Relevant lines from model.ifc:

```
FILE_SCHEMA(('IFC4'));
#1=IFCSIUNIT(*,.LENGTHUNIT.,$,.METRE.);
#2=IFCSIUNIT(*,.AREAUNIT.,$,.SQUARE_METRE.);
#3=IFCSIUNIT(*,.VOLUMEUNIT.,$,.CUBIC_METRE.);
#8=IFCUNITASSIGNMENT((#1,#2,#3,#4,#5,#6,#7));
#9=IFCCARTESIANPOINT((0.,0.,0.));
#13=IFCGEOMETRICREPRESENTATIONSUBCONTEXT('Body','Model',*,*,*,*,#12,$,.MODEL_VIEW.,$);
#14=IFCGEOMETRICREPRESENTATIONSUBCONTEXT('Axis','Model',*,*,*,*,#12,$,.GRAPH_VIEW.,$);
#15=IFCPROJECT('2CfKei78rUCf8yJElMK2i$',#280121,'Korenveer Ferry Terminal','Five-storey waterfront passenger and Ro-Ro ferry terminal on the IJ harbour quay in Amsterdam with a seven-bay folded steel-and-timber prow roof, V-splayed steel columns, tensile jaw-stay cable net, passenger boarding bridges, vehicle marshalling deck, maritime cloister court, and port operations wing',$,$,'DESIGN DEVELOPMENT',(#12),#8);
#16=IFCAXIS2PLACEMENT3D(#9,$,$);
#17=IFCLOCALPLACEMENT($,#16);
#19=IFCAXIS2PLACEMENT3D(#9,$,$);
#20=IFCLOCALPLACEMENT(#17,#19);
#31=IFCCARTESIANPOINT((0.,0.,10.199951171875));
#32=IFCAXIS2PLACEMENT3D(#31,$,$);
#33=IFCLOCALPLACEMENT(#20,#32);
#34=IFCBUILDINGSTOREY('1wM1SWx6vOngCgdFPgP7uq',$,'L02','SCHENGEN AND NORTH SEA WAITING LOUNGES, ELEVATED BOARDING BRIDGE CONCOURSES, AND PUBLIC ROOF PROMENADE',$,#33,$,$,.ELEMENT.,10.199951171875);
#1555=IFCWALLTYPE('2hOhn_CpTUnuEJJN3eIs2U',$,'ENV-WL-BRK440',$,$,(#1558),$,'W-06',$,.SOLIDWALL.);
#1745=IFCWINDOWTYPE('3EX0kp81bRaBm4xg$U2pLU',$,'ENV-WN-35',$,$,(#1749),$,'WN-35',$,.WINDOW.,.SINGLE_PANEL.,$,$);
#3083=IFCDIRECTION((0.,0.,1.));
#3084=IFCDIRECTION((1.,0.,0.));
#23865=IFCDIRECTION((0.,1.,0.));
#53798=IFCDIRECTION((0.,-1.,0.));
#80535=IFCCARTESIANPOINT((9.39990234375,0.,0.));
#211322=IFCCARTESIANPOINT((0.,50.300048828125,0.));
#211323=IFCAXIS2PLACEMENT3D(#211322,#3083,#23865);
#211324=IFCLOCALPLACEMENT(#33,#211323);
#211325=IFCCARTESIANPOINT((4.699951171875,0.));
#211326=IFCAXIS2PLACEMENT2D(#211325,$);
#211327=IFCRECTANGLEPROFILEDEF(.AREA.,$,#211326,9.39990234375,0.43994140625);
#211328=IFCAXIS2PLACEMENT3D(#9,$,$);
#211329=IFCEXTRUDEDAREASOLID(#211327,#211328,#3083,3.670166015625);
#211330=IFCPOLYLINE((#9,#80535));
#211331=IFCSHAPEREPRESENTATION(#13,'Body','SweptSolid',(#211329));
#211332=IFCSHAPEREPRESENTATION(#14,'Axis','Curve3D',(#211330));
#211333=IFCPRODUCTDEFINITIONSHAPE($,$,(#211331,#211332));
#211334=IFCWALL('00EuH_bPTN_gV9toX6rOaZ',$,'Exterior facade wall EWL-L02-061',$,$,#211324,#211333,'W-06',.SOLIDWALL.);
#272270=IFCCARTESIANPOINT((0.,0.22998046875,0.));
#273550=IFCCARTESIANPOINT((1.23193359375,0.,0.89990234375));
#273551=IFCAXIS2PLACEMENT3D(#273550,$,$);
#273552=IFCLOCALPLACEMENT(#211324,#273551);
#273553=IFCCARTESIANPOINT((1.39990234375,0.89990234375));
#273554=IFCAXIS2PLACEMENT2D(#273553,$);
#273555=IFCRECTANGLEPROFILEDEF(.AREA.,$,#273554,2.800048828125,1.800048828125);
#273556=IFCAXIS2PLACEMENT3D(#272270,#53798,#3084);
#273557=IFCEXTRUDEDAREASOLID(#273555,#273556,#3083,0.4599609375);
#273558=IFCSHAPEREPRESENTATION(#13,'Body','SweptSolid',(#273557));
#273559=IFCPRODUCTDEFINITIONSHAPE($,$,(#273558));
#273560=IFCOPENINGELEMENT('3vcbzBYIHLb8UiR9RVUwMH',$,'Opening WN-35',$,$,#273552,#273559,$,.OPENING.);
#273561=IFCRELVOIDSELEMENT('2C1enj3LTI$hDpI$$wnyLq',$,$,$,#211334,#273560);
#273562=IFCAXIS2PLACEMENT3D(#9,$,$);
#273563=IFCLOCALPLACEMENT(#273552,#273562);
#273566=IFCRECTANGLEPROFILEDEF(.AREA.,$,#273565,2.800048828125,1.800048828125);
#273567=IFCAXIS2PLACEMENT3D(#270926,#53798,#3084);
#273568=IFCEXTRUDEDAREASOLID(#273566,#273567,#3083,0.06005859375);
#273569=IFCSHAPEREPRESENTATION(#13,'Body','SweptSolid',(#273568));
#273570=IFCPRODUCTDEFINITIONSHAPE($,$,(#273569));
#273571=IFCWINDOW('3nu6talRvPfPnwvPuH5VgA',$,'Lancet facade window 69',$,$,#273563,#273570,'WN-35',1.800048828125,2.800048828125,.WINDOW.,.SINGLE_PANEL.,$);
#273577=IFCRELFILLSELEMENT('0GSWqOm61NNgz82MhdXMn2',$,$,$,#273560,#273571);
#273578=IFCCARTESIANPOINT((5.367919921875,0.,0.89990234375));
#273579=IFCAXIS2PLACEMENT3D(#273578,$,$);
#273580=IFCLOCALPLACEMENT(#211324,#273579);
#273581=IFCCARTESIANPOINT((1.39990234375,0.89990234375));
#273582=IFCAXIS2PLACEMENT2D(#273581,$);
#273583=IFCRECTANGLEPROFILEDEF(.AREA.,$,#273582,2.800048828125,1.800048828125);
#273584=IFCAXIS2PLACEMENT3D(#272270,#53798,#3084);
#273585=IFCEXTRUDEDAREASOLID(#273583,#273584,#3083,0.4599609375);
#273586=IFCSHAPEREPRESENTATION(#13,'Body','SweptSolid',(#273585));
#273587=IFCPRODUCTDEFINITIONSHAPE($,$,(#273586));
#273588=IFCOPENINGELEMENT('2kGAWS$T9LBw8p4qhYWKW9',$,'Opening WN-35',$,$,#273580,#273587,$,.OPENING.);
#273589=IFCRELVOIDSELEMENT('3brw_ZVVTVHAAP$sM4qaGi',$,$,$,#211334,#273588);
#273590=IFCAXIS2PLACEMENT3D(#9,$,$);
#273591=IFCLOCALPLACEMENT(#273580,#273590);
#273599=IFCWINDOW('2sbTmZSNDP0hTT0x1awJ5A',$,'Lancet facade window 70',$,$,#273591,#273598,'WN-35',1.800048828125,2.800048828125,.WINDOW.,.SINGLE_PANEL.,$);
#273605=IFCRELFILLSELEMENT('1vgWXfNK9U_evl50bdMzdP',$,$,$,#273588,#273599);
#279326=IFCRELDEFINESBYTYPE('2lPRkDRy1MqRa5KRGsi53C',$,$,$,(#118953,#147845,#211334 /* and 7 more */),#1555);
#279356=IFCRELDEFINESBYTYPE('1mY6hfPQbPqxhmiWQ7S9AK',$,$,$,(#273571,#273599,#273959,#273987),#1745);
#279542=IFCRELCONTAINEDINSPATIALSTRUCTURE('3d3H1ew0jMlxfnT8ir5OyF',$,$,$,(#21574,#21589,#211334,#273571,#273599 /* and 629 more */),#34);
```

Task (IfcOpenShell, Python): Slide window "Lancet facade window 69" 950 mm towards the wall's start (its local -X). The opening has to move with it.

```python
import ifcopenshell
import ifcopenshell.api.geometry
import ifcopenshell.util.placement

model = ifcopenshell.open("model.ifc")

window = model.by_id(273571)
opening = window.FillsVoids[0].RelatingOpeningElement
wall = opening.VoidsElements[0].RelatingBuildingElement

wall_matrix = ifcopenshell.util.placement.get_local_placement(wall.ObjectPlacement)
shift = wall_matrix[:3, 0] * -0.95
before = ifcopenshell.util.placement.get_local_placement(window.ObjectPlacement)[:3, 3].copy()

# The window is placed relative to its opening, so it follows when the opening moves.
matrix = ifcopenshell.util.placement.get_local_placement(opening.ObjectPlacement)
matrix[:3, 3] += shift
ifcopenshell.api.geometry.edit_object_placement(
    model, product=opening, matrix=matrix, is_si=False, should_transform_children=True
)

after = ifcopenshell.util.placement.get_local_placement(window.ObjectPlacement)[:3, 3]
print("window moved by", (after - before).round(3) + 0.0)

model.write("model_v2.ifc")
```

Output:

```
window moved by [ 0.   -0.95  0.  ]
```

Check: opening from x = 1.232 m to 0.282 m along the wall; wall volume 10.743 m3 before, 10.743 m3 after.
